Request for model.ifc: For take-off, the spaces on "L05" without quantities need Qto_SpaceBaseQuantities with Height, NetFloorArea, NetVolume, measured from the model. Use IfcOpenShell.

First a look at what the model holds.

```python
import ifcopenshell
import ifcopenshell.util.element
import ifcopenshell.util.unit

model = ifcopenshell.open("model.ifc")
print(model.schema)
for unit_type in ("LENGTHUNIT", "AREAUNIT", "VOLUMEUNIT"):
    print(unit_type, ifcopenshell.util.unit.calculate_unit_scale(model, unit_type))
storey = next(s for s in model.by_type("IfcBuildingStorey") if s.Name == "L05")
spaces = [e for e in ifcopenshell.util.element.get_decomposition(storey) if e.is_a("IfcSpace")]
for e in sorted(spaces, key=lambda e: e.id()):
    print(e.id(), e.is_a(), e.Name, list(ifcopenshell.util.element.get_psets(e, qtos_only=True)), sep=" | ")
```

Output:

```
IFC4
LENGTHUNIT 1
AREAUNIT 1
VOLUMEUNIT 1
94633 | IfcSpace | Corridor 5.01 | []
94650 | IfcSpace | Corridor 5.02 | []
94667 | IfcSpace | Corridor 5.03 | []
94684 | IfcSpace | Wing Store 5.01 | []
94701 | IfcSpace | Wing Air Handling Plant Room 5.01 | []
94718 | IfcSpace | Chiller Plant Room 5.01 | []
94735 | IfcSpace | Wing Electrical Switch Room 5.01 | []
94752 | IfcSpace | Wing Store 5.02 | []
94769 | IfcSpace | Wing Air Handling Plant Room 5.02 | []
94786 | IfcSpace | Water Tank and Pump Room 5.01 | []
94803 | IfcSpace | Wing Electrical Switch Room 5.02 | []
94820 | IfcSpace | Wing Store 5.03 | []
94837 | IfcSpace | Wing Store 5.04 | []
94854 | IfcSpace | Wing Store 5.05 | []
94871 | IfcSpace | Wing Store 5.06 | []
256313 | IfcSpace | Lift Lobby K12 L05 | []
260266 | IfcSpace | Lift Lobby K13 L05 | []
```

```python
import ifcopenshell
import ifcopenshell.api.pset
import ifcopenshell.geom
import ifcopenshell.util.element
import ifcopenshell.util.shape
import ifcopenshell.util.unit

model = ifcopenshell.open("model.ifc")
unit_scale = ifcopenshell.util.unit.calculate_unit_scale(model)
area_scale = ifcopenshell.util.unit.calculate_unit_scale(model, "AREAUNIT")
volume_scale = ifcopenshell.util.unit.calculate_unit_scale(model, "VOLUMEUNIT")
settings = ifcopenshell.geom.settings()

storey = next(s for s in model.by_type("IfcBuildingStorey") if s.Name == "L05")
spaces = [e for e in ifcopenshell.util.element.get_decomposition(storey) if e.is_a("IfcSpace")]

for e in sorted(spaces, key=lambda e: e.id()):
    if ifcopenshell.util.element.get_psets(e, qtos_only=True, should_inherit=False):
        continue
    # Geometry comes back in metres, in the element's own axes.
    shape = ifcopenshell.geom.create_shape(settings, e)
    values = {
        "Height": ifcopenshell.util.shape.get_z(shape.geometry) / unit_scale,
        "NetFloorArea": ifcopenshell.util.shape.get_footprint_area(shape.geometry) / area_scale,
        "NetVolume": ifcopenshell.util.shape.get_volume(shape.geometry) / volume_scale,
    }
    qto = ifcopenshell.api.pset.add_qto(model, product=e, name="Qto_SpaceBaseQuantities")
    ifcopenshell.api.pset.edit_qto(model, qto=qto, properties=values)
    print(e.id(), {k: round(v, 3) for k, v in values.items()})

model.write("model_edited.ifc")
```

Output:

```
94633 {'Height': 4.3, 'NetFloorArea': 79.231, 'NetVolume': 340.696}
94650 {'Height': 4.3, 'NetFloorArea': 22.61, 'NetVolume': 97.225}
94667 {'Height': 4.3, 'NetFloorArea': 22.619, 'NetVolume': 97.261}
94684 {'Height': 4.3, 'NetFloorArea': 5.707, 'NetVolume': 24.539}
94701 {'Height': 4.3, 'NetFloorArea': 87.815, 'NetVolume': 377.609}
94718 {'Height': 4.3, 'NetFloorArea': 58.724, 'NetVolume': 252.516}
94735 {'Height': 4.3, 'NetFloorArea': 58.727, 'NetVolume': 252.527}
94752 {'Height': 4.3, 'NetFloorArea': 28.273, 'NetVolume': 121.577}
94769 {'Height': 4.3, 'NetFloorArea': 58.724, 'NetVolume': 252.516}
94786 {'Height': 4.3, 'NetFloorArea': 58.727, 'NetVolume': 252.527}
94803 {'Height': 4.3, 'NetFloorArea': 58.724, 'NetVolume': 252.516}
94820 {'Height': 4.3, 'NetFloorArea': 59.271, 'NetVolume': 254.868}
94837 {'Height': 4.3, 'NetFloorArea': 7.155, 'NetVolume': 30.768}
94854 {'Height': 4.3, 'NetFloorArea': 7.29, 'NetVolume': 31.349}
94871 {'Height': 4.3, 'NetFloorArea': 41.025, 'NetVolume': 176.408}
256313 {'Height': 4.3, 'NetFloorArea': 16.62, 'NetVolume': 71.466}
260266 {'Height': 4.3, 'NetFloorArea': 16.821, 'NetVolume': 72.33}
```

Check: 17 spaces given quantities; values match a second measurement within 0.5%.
